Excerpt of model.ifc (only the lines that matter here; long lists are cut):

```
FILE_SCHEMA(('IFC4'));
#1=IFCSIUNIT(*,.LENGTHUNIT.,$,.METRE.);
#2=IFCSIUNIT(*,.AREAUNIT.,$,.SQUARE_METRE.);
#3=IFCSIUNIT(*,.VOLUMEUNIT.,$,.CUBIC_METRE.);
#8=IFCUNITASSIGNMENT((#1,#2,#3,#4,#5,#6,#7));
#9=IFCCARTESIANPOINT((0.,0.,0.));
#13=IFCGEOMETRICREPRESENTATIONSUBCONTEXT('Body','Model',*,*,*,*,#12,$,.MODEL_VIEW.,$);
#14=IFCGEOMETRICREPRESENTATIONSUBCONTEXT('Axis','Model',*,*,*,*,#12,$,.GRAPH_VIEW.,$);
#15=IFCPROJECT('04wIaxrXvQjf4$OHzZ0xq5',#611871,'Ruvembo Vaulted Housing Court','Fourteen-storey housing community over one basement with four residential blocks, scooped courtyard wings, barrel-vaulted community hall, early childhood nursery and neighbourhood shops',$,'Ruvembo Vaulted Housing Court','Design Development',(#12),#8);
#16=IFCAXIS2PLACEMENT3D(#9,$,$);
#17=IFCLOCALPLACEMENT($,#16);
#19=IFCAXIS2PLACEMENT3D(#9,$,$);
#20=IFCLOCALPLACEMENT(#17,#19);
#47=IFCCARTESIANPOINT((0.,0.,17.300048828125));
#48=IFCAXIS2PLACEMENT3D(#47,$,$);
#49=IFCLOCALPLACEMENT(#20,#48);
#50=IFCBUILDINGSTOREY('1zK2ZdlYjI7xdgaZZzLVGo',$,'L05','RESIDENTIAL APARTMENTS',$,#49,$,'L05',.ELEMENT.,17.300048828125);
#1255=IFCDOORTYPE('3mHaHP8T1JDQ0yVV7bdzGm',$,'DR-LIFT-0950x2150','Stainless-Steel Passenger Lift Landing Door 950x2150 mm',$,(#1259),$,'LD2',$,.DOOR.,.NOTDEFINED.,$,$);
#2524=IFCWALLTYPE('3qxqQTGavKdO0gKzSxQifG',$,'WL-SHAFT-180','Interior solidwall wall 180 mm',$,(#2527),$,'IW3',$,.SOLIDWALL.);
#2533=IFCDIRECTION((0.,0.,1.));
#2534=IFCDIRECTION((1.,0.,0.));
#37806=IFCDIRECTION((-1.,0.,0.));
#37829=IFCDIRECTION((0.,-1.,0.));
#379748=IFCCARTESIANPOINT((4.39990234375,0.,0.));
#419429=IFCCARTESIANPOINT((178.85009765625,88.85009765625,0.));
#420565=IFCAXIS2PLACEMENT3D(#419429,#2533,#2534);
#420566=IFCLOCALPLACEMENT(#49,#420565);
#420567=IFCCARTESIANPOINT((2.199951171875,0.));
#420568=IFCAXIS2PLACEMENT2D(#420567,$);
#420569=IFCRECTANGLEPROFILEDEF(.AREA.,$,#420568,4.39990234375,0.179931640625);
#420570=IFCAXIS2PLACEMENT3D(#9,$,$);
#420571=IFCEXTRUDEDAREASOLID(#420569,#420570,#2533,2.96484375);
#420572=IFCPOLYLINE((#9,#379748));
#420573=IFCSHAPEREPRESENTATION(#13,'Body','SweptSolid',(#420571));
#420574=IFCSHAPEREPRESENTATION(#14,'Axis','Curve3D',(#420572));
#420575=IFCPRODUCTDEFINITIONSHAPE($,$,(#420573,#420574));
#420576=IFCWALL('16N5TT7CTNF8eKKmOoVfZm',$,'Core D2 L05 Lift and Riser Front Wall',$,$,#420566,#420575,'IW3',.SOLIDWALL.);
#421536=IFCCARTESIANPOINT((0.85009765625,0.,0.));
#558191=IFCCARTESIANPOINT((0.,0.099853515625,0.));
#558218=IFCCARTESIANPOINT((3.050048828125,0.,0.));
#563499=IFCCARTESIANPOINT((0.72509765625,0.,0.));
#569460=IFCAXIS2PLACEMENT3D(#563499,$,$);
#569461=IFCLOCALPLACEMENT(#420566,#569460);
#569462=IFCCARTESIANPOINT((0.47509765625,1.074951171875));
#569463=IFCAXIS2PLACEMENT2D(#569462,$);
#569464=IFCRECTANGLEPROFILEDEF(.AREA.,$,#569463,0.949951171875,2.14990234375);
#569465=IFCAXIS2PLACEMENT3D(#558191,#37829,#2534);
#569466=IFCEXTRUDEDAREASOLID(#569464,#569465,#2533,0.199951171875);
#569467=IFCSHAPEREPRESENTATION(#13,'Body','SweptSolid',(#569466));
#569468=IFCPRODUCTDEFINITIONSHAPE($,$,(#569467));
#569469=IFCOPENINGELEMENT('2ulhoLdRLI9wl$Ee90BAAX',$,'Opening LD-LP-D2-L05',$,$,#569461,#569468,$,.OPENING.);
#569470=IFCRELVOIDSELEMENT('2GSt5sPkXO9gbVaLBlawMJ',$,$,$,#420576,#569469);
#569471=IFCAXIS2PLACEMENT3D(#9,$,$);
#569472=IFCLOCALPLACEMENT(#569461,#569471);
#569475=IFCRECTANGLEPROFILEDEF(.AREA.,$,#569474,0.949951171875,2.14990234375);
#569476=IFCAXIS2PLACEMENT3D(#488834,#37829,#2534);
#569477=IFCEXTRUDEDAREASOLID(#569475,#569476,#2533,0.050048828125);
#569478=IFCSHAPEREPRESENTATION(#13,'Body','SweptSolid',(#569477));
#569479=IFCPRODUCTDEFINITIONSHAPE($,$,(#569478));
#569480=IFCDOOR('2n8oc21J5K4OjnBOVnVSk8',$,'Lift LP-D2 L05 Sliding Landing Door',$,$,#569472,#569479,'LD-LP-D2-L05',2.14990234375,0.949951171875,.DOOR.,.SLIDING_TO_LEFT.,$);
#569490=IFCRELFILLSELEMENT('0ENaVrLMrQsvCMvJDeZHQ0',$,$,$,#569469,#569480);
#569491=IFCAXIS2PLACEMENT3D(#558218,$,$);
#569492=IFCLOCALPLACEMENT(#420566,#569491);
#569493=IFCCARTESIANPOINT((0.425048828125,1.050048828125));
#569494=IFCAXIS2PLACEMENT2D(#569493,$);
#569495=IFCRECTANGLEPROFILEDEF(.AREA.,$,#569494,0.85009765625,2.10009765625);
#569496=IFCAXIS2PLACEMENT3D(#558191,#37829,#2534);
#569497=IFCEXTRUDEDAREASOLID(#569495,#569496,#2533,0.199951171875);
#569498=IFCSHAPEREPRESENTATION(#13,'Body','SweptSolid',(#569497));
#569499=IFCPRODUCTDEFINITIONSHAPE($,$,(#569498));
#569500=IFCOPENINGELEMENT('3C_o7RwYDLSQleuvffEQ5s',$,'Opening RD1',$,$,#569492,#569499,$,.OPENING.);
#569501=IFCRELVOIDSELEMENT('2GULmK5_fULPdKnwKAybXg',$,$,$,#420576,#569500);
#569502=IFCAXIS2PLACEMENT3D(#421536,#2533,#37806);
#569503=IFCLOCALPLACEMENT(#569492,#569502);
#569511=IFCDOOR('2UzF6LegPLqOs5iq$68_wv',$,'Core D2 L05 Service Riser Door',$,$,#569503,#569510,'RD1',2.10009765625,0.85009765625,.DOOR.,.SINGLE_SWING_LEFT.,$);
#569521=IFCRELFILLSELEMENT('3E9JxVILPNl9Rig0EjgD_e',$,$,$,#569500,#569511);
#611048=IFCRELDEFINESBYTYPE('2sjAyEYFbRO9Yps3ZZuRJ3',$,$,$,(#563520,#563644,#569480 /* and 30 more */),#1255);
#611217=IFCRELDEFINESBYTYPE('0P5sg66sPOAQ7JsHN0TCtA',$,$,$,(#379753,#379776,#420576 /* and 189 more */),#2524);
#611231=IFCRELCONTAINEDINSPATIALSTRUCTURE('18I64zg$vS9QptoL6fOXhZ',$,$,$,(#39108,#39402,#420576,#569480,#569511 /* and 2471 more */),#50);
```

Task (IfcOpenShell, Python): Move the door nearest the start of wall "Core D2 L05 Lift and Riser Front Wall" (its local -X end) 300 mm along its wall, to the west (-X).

```python
import ifcopenshell
import ifcopenshell.api.geometry
import ifcopenshell.util.placement
import ifcopenshell.util.unit

model = ifcopenshell.open("model.ifc")
unit_scale = ifcopenshell.util.unit.calculate_unit_scale(model)

door = model.by_guid("2n8oc21J5K4OjnBOVnVSk8")
opening = door.FillsVoids[0].RelatingOpeningElement
wall = opening.VoidsElements[0].RelatingBuildingElement

wall_matrix = ifcopenshell.util.placement.get_local_placement(wall.ObjectPlacement)
shift = wall_matrix[:3, 0] * -0.3 / unit_scale
before = ifcopenshell.util.placement.get_local_placement(door.ObjectPlacement)[:3, 3].copy()

# The door is placed relative to its opening, so it follows when the opening moves.
matrix = ifcopenshell.util.placement.get_local_placement(opening.ObjectPlacement)
matrix[:3, 3] += shift
ifcopenshell.api.geometry.edit_object_placement(
    model, product=opening, matrix=matrix, is_si=False, should_transform_children=True
)

after = ifcopenshell.util.placement.get_local_placement(door.ObjectPlacement)[:3, 3]
print("door moved by", (after - before).round(3) + 0.0)

model.write("model_updated.ifc")
```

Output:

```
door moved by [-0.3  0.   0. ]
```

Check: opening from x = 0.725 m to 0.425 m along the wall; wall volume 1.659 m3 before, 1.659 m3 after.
